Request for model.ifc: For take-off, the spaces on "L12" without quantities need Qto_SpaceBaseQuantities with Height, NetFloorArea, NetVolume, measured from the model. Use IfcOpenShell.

First a look at what the model holds.

```python
import ifcopenshell
import ifcopenshell.util.element
import ifcopenshell.util.unit

model = ifcopenshell.open("model.ifc")
print(model.schema)
for unit_type in ("LENGTHUNIT", "AREAUNIT", "VOLUMEUNIT"):
    print(unit_type, ifcopenshell.util.unit.calculate_unit_scale(model, unit_type))
storey = next(s for s in model.by_type("IfcBuildingStorey") if s.Name == "L12")
spaces = [e for e in ifcopenshell.util.element.get_decomposition(storey) if e.is_a("IfcSpace")]
for e in sorted(spaces, key=lambda e: e.id()):
    print(e.id(), e.is_a(), e.Name, list(ifcopenshell.util.element.get_psets(e, qtos_only=True)), sep=" | ")
```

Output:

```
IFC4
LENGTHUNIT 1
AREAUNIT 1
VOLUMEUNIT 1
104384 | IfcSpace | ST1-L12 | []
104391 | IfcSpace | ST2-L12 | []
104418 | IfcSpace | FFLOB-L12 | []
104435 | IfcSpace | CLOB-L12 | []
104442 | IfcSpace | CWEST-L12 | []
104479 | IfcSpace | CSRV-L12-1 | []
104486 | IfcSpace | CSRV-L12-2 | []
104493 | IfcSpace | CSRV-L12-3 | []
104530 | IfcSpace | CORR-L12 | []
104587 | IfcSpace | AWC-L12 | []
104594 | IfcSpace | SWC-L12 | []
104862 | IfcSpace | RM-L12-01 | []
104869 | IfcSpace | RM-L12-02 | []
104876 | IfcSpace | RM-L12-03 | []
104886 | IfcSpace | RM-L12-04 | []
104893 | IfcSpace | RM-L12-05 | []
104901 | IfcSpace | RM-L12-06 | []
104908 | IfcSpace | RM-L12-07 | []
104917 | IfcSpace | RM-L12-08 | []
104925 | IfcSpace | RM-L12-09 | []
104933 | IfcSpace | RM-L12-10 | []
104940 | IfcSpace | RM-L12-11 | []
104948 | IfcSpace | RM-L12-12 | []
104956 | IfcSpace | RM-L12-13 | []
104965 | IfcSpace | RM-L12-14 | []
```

```python
import ifcopenshell
import ifcopenshell.api.pset
import ifcopenshell.geom
import ifcopenshell.util.element
import ifcopenshell.util.shape
import ifcopenshell.util.unit

model = ifcopenshell.open("model.ifc")
unit_scale = ifcopenshell.util.unit.calculate_unit_scale(model)
area_scale = ifcopenshell.util.unit.calculate_unit_scale(model, "AREAUNIT")
volume_scale = ifcopenshell.util.unit.calculate_unit_scale(model, "VOLUMEUNIT")
settings = ifcopenshell.geom.settings()

storey = next(s for s in model.by_type("IfcBuildingStorey") if s.Name == "L12")
spaces = [e for e in ifcopenshell.util.element.get_decomposition(storey) if e.is_a("IfcSpace")]

for e in sorted(spaces, key=lambda e: e.id()):
    if ifcopenshell.util.element.get_psets(e, qtos_only=True, should_inherit=False):
        continue
    # Geometry comes back in metres, in the element's own axes.
    shape = ifcopenshell.geom.create_shape(settings, e)
    values = {
        "Height": ifcopenshell.util.shape.get_z(shape.geometry) / unit_scale,
        "NetFloorArea": ifcopenshell.util.shape.get_footprint_area(shape.geometry) / area_scale,
        "NetVolume": ifcopenshell.util.shape.get_volume(shape.geometry) / volume_scale,
    }
    qto = ifcopenshell.api.pset.add_qto(model, product=e, name="Qto_SpaceBaseQuantities")
    ifcopenshell.api.pset.edit_qto(model, qto=qto, properties=values)
    print(e.id(), {k: round(v, 3) for k, v in values.items()})

model.write("model_v2.ifc")
```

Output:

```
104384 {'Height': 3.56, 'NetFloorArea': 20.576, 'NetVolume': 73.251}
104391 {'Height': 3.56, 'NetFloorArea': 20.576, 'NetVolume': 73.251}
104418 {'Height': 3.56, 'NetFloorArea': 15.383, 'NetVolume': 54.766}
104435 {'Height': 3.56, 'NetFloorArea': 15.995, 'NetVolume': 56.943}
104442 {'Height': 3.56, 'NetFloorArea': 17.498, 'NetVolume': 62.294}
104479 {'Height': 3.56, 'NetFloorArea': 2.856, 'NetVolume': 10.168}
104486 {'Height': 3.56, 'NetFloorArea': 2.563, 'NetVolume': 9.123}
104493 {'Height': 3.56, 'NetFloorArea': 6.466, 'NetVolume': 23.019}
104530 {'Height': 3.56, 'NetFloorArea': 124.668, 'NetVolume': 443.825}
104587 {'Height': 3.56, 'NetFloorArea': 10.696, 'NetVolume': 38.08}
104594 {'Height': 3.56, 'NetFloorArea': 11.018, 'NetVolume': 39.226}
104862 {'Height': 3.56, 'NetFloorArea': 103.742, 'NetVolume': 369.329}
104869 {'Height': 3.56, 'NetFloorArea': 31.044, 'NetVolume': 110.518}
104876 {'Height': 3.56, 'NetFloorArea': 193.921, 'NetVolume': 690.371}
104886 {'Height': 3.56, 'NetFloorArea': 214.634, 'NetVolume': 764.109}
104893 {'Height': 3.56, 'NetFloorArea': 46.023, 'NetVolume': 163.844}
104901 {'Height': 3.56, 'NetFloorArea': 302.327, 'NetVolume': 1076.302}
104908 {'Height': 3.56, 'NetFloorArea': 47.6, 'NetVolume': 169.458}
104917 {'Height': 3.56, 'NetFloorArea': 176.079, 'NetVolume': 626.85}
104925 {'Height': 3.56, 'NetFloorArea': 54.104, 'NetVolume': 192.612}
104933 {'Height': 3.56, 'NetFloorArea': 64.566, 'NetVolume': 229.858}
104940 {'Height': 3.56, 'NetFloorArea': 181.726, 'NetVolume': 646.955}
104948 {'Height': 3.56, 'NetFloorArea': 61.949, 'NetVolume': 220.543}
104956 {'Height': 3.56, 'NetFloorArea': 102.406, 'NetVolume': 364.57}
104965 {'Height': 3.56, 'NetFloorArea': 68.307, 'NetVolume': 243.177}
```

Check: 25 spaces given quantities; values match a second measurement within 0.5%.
